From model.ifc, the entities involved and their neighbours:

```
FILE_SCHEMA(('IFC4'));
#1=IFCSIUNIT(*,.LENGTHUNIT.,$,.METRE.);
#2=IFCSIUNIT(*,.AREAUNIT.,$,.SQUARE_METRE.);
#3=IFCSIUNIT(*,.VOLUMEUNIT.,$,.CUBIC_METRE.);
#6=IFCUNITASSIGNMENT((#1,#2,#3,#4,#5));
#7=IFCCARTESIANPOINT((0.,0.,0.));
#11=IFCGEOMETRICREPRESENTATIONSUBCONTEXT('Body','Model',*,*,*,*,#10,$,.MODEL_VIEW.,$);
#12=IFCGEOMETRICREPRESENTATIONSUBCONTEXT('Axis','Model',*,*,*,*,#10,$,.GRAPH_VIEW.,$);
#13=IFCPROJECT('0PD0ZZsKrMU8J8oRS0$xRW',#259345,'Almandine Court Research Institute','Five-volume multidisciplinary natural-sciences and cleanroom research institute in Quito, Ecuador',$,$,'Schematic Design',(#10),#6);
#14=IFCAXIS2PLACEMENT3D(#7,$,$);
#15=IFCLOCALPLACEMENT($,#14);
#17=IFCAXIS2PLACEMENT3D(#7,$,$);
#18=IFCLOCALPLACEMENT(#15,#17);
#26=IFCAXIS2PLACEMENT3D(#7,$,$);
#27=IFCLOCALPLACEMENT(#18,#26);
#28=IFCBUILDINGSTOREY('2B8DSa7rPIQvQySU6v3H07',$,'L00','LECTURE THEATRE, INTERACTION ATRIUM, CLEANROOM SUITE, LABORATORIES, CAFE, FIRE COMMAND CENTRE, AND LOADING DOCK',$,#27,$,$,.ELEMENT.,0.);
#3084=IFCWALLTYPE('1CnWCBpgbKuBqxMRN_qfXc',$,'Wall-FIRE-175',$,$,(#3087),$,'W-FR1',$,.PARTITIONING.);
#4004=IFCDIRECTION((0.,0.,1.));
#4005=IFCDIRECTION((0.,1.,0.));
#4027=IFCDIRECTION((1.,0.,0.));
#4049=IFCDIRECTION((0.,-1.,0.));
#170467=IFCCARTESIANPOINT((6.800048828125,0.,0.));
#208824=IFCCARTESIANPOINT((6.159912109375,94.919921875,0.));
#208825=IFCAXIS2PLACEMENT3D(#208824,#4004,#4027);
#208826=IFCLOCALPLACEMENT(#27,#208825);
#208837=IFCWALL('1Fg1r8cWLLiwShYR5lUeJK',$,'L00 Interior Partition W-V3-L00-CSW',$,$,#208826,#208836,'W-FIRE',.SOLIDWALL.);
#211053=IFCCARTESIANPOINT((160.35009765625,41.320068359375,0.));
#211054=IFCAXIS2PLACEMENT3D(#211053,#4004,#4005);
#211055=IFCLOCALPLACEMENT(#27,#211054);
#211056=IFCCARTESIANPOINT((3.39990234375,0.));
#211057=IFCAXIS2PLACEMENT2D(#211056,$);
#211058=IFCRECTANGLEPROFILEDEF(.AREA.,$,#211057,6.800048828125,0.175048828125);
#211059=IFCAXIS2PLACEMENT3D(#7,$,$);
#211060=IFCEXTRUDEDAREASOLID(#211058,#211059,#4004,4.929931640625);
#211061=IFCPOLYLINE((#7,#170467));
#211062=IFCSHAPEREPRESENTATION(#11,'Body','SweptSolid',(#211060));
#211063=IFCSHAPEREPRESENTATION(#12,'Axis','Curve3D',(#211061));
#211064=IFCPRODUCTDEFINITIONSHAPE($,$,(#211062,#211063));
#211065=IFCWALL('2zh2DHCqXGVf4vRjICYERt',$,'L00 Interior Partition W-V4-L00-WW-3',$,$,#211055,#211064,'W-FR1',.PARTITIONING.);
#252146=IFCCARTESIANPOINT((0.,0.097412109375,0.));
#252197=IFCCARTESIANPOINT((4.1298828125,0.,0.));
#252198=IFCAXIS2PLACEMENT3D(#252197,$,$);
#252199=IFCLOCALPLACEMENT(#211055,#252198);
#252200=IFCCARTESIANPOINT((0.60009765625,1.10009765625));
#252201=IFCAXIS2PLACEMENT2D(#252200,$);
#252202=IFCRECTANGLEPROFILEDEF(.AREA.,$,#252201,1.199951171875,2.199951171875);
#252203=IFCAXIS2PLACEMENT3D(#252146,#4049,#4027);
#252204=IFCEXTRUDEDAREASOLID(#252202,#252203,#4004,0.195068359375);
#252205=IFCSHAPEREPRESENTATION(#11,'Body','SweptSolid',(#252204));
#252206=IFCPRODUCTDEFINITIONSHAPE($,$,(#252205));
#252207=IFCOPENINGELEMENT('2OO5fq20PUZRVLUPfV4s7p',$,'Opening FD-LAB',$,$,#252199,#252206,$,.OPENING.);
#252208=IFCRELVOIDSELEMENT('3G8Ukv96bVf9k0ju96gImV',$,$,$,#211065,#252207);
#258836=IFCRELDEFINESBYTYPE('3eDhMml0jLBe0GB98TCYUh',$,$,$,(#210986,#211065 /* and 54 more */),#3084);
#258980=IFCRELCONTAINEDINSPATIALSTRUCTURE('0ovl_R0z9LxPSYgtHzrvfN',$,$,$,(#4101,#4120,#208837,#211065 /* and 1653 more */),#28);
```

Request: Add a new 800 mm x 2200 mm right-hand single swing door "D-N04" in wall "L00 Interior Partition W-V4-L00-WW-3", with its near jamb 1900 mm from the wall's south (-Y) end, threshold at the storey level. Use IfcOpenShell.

```python
import numpy as np
import ifcopenshell
import ifcopenshell.api.feature
import ifcopenshell.api.geometry
import ifcopenshell.api.root
import ifcopenshell.api.spatial
import ifcopenshell.geom
import ifcopenshell.util.element
import ifcopenshell.util.placement
import ifcopenshell.util.representation
import ifcopenshell.util.shape
import ifcopenshell.util.unit

model = ifcopenshell.open("model.ifc")
unit_scale = ifcopenshell.util.unit.calculate_unit_scale(model)
settings = ifcopenshell.geom.settings()


def volume(element):
    """Net volume in cubic metres, openings subtracted."""
    shape = ifcopenshell.geom.create_shape(settings, element)
    return ifcopenshell.util.shape.get_volume(shape.geometry)


wall = model.by_guid("2zh2DHCqXGVf4vRjICYERt")
storey = ifcopenshell.util.element.get_container(wall, ifc_class="IfcBuildingStorey")
context = ifcopenshell.util.representation.get_context(model, "Model", "Body", "MODEL_VIEW")
before = volume(wall)

width, height, from_end, sill = 0.8, 2.2, 1.9, 0.0  # metres

# The wall runs along its own X axis, and the end named is its -X end.
wall_shape = ifcopenshell.geom.create_shape(settings, wall)
x, y, z = ifcopenshell.util.shape.get_vertices(wall_shape.geometry).T
start = x.min() + from_end
face, thickness = float(y.min()), float(y.max() - y.min())
wall_matrix = ifcopenshell.util.placement.get_local_placement(wall.ObjectPlacement)
level = ifcopenshell.util.placement.get_local_placement(storey.ObjectPlacement)[2, 3]


def in_wall(x, y):
    """Placement at x, y metres in the wall's axes, at sill height."""
    matrix = wall_matrix.copy()
    matrix[:, 3] = wall_matrix @ np.array([x / unit_scale, y / unit_scale, 0.0, 1.0])
    matrix[2, 3] = level + sill / unit_scale
    return matrix


# Opening: a box that overshoots both wall faces by 50 mm.
opening = ifcopenshell.api.root.create_entity(model, ifc_class="IfcOpeningElement", predefined_type="OPENING")
box = ifcopenshell.api.geometry.add_wall_representation(
    model, context=context, length=width, height=height, thickness=thickness + 0.1
)
ifcopenshell.api.geometry.assign_representation(model, product=opening, representation=box)
ifcopenshell.api.geometry.edit_object_placement(model, product=opening, matrix=in_wall(start, face - 0.05), is_si=False)
ifcopenshell.api.feature.add_feature(model, feature=opening, element=wall)

door = ifcopenshell.api.root.create_entity(model, ifc_class="IfcDoor", name="D-N04", predefined_type="DOOR")
door.OverallWidth, door.OverallHeight = width / unit_scale, height / unit_scale
door.OperationType = "SINGLE_SWING_RIGHT"
body = ifcopenshell.api.geometry.add_door_representation(
    model,
    context=context,
    overall_width=door.OverallWidth,
    overall_height=door.OverallHeight,
    operation_type="SINGLE_SWING_RIGHT",
    lining_properties={"LiningDepth": thickness / unit_scale, "ThresholdDepth": thickness / unit_scale},
)
ifcopenshell.api.geometry.assign_representation(model, product=door, representation=body)
ifcopenshell.api.spatial.assign_container(model, products=[door], relating_structure=storey)
ifcopenshell.api.feature.add_filling(model, opening=opening, element=door)

# The lining spans the wall, so the door starts at the wall face.
ifcopenshell.api.geometry.edit_object_placement(model, product=door, matrix=in_wall(start, face), is_si=False)

after = volume(wall)

print(f"wall volume {before:.3f} -> {after:.3f} m3")

model.write("model-out.ifc")
```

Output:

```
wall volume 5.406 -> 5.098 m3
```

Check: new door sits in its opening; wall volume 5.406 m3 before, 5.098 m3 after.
